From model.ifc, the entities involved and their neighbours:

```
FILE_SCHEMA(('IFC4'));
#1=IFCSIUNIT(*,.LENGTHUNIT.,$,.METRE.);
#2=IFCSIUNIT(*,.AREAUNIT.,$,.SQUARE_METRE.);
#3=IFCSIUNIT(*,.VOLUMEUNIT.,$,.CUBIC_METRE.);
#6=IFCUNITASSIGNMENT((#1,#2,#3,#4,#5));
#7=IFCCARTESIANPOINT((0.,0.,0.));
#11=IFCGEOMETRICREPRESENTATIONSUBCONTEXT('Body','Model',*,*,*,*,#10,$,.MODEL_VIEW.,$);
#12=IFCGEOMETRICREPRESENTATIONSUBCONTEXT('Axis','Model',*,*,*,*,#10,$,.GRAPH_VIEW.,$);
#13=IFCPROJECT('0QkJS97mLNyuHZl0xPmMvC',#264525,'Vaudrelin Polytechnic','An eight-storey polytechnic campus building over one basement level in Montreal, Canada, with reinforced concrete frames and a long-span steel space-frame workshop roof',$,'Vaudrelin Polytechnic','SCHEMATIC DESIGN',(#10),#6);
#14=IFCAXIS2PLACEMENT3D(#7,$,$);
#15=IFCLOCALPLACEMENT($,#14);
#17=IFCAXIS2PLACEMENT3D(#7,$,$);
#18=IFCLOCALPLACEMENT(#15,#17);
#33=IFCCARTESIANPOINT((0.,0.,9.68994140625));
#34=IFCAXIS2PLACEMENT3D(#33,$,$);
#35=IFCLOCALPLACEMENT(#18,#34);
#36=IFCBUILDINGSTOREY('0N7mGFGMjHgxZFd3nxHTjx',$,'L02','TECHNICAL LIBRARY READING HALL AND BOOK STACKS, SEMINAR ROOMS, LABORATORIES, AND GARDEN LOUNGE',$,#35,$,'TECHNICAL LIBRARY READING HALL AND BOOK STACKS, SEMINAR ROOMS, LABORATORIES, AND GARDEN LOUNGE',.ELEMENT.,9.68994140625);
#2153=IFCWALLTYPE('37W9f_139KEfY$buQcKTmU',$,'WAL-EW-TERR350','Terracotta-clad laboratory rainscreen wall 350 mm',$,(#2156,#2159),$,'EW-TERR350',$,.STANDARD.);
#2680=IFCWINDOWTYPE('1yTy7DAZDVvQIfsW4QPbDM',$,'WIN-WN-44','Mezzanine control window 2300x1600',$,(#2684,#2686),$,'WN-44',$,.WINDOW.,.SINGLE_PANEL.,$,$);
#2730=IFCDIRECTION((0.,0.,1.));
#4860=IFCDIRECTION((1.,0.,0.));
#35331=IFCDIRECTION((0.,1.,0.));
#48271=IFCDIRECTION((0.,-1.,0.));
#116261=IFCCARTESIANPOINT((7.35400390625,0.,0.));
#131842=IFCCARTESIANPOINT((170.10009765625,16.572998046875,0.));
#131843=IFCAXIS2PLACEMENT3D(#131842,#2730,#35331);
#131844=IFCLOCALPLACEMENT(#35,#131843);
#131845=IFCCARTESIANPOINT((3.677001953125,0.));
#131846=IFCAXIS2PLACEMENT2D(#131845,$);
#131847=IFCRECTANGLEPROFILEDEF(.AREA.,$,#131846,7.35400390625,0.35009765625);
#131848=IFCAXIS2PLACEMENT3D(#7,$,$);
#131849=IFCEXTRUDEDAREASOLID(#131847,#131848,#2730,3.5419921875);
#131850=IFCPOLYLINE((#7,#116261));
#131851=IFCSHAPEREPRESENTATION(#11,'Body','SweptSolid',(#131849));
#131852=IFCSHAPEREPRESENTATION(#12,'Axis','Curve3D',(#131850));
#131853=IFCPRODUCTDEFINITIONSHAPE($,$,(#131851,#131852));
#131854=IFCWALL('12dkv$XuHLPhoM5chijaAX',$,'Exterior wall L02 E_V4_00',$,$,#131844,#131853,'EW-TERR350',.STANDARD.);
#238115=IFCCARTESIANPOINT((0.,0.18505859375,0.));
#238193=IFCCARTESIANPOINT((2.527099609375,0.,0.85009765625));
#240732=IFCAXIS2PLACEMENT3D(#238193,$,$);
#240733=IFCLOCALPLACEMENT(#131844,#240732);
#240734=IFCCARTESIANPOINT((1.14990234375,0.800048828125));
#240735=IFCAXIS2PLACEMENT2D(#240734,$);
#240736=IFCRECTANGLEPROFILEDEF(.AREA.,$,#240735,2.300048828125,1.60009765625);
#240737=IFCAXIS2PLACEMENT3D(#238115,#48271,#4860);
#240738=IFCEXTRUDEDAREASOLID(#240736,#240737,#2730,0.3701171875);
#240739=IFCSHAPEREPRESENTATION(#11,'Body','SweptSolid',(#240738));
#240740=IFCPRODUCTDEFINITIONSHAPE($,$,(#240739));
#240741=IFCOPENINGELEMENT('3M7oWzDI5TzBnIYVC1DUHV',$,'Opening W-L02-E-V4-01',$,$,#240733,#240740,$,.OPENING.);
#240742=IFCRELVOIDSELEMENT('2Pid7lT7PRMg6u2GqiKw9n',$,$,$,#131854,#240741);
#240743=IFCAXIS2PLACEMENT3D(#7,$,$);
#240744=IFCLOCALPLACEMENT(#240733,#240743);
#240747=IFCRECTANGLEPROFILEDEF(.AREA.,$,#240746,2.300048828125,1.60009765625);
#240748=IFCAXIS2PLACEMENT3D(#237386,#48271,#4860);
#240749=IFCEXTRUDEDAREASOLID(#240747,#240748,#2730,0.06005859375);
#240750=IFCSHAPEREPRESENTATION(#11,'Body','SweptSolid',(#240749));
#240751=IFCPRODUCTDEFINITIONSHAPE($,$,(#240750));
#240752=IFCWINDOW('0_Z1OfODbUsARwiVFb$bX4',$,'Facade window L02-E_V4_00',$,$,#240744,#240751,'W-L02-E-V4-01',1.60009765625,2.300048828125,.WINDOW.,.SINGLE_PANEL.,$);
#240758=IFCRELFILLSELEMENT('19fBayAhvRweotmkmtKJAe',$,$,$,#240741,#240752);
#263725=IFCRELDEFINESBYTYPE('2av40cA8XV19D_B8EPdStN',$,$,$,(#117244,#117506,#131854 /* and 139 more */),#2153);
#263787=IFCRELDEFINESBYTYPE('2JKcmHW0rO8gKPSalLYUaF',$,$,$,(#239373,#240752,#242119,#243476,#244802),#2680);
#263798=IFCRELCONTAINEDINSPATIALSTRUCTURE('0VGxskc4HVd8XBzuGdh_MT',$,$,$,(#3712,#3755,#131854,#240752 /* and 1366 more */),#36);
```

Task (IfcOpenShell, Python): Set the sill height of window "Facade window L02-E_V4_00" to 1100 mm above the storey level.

```python
import numpy as np
import ifcopenshell
import ifcopenshell.api.geometry
import ifcopenshell.geom
import ifcopenshell.util.element
import ifcopenshell.util.placement
import ifcopenshell.util.shape
import ifcopenshell.util.unit

model = ifcopenshell.open("model.ifc")
unit_scale = ifcopenshell.util.unit.calculate_unit_scale(model)

window = model.by_guid("0_Z1OfODbUsARwiVFb$bX4")
opening = window.FillsVoids[0].RelatingOpeningElement
storey = ifcopenshell.util.element.get_container(window, ifc_class="IfcBuildingStorey")
level = ifcopenshell.util.placement.get_local_placement(storey.ObjectPlacement)[2, 3]

# The opening's origin need not be at the sill, so measure its lowest point.
shape = ifcopenshell.geom.create_shape(ifcopenshell.geom.settings(), opening)
bottom = ifcopenshell.util.shape.get_shape_bottom_elevation(shape, shape.geometry) / unit_scale
dz = level + 1.1 / unit_scale - bottom

shift = np.array([0.0, 0.0, dz])
# The window is placed relative to its opening, so it follows when the opening moves.
matrix = ifcopenshell.util.placement.get_local_placement(opening.ObjectPlacement)
matrix[:3, 3] += shift
ifcopenshell.api.geometry.edit_object_placement(
    model, product=opening, matrix=matrix, is_si=False, should_transform_children=True
)

print(f"moved by {dz * unit_scale:+.3f} m")

model.write("model_rev.ifc")
```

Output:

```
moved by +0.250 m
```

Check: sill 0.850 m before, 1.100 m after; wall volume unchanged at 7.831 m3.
